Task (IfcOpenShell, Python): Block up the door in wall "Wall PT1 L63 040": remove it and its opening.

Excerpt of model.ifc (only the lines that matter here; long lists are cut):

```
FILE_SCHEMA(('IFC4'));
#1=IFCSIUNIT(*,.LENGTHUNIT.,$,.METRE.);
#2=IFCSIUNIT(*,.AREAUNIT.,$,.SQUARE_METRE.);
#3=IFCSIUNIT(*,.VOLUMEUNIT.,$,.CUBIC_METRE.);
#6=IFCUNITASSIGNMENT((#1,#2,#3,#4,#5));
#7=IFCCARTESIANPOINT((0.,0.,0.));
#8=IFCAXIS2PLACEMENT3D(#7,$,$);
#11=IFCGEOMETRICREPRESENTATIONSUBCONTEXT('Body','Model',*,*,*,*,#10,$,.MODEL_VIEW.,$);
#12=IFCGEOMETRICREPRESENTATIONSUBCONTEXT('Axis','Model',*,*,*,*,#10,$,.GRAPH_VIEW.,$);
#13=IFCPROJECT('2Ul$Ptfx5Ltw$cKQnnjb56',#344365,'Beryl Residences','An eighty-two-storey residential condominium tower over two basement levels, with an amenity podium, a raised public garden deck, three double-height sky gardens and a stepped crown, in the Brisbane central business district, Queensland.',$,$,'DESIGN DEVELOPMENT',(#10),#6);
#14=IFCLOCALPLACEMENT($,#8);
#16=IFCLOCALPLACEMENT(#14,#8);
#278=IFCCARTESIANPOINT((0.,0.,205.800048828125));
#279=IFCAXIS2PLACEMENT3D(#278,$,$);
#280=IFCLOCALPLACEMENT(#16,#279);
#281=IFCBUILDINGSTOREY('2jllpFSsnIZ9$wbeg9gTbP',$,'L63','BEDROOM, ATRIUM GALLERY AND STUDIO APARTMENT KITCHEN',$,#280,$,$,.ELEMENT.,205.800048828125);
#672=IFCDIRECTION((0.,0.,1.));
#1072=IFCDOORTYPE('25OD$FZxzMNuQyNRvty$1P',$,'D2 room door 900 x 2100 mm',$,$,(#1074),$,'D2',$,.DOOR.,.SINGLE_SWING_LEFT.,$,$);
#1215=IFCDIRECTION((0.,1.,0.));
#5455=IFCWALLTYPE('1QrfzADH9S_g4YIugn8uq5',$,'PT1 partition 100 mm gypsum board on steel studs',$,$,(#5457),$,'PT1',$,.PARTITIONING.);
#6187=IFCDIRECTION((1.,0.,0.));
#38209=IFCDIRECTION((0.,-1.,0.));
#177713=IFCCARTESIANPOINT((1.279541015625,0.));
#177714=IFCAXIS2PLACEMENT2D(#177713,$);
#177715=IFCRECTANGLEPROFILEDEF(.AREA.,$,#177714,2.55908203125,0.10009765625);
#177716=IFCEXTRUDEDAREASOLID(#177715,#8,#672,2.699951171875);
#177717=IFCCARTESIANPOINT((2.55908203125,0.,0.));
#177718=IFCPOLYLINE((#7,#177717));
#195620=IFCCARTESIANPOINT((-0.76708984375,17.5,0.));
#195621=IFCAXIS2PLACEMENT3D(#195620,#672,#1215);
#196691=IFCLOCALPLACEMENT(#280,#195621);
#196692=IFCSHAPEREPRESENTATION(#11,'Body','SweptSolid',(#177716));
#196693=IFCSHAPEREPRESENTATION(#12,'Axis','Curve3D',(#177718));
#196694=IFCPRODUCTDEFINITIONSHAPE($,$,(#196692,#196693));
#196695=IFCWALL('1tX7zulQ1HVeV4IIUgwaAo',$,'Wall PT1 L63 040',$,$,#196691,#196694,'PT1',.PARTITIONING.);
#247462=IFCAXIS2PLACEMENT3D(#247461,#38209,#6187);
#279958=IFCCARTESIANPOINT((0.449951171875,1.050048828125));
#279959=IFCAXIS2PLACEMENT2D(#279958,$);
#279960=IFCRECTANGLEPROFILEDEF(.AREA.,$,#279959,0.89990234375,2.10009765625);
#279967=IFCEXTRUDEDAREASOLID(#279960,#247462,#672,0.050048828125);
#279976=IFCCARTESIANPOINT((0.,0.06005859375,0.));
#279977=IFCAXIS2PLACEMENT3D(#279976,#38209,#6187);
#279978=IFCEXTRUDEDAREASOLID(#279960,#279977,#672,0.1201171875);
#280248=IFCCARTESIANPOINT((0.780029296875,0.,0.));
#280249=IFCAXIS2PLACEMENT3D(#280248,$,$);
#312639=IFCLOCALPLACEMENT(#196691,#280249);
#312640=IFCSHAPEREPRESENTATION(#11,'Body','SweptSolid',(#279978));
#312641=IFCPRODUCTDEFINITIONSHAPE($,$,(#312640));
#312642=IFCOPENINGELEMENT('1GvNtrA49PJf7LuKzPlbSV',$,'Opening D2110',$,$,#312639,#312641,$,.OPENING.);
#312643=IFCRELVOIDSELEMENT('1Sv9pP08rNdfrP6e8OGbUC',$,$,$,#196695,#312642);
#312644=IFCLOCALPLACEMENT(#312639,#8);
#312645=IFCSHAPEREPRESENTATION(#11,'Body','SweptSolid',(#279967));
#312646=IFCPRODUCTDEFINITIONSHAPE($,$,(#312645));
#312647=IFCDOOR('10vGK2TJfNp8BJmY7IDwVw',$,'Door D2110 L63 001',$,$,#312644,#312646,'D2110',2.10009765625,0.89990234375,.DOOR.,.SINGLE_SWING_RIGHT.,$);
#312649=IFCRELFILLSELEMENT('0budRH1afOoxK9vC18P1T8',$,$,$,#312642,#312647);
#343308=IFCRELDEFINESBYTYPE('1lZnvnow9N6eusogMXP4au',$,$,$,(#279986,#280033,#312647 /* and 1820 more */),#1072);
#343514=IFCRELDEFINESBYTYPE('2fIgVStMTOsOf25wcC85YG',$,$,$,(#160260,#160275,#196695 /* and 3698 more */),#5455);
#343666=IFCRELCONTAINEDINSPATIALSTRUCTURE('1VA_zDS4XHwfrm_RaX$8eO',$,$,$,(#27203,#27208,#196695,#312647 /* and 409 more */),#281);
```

```python
import ifcopenshell
import ifcopenshell.api.feature
import ifcopenshell.api.root
import ifcopenshell.geom
import ifcopenshell.util.shape

model = ifcopenshell.open("model.ifc")
settings = ifcopenshell.geom.settings()


def volume(element):
    """Net volume in cubic metres, openings subtracted."""
    shape = ifcopenshell.geom.create_shape(settings, element)
    return ifcopenshell.util.shape.get_volume(shape.geometry)


door = model.by_guid("10vGK2TJfNp8BJmY7IDwVw")
opening = door.FillsVoids[0].RelatingOpeningElement
wall = opening.VoidsElements[0].RelatingBuildingElement
before = volume(wall)

ifcopenshell.api.root.remove_product(model, product=door)
ifcopenshell.api.feature.remove_feature(model, feature=opening)

after = volume(wall)

print(f"wall volume {before:.3f} -> {after:.3f} m3")

model.write("model_edited.ifc")
```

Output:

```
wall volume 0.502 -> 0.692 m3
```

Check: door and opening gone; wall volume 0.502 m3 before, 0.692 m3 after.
